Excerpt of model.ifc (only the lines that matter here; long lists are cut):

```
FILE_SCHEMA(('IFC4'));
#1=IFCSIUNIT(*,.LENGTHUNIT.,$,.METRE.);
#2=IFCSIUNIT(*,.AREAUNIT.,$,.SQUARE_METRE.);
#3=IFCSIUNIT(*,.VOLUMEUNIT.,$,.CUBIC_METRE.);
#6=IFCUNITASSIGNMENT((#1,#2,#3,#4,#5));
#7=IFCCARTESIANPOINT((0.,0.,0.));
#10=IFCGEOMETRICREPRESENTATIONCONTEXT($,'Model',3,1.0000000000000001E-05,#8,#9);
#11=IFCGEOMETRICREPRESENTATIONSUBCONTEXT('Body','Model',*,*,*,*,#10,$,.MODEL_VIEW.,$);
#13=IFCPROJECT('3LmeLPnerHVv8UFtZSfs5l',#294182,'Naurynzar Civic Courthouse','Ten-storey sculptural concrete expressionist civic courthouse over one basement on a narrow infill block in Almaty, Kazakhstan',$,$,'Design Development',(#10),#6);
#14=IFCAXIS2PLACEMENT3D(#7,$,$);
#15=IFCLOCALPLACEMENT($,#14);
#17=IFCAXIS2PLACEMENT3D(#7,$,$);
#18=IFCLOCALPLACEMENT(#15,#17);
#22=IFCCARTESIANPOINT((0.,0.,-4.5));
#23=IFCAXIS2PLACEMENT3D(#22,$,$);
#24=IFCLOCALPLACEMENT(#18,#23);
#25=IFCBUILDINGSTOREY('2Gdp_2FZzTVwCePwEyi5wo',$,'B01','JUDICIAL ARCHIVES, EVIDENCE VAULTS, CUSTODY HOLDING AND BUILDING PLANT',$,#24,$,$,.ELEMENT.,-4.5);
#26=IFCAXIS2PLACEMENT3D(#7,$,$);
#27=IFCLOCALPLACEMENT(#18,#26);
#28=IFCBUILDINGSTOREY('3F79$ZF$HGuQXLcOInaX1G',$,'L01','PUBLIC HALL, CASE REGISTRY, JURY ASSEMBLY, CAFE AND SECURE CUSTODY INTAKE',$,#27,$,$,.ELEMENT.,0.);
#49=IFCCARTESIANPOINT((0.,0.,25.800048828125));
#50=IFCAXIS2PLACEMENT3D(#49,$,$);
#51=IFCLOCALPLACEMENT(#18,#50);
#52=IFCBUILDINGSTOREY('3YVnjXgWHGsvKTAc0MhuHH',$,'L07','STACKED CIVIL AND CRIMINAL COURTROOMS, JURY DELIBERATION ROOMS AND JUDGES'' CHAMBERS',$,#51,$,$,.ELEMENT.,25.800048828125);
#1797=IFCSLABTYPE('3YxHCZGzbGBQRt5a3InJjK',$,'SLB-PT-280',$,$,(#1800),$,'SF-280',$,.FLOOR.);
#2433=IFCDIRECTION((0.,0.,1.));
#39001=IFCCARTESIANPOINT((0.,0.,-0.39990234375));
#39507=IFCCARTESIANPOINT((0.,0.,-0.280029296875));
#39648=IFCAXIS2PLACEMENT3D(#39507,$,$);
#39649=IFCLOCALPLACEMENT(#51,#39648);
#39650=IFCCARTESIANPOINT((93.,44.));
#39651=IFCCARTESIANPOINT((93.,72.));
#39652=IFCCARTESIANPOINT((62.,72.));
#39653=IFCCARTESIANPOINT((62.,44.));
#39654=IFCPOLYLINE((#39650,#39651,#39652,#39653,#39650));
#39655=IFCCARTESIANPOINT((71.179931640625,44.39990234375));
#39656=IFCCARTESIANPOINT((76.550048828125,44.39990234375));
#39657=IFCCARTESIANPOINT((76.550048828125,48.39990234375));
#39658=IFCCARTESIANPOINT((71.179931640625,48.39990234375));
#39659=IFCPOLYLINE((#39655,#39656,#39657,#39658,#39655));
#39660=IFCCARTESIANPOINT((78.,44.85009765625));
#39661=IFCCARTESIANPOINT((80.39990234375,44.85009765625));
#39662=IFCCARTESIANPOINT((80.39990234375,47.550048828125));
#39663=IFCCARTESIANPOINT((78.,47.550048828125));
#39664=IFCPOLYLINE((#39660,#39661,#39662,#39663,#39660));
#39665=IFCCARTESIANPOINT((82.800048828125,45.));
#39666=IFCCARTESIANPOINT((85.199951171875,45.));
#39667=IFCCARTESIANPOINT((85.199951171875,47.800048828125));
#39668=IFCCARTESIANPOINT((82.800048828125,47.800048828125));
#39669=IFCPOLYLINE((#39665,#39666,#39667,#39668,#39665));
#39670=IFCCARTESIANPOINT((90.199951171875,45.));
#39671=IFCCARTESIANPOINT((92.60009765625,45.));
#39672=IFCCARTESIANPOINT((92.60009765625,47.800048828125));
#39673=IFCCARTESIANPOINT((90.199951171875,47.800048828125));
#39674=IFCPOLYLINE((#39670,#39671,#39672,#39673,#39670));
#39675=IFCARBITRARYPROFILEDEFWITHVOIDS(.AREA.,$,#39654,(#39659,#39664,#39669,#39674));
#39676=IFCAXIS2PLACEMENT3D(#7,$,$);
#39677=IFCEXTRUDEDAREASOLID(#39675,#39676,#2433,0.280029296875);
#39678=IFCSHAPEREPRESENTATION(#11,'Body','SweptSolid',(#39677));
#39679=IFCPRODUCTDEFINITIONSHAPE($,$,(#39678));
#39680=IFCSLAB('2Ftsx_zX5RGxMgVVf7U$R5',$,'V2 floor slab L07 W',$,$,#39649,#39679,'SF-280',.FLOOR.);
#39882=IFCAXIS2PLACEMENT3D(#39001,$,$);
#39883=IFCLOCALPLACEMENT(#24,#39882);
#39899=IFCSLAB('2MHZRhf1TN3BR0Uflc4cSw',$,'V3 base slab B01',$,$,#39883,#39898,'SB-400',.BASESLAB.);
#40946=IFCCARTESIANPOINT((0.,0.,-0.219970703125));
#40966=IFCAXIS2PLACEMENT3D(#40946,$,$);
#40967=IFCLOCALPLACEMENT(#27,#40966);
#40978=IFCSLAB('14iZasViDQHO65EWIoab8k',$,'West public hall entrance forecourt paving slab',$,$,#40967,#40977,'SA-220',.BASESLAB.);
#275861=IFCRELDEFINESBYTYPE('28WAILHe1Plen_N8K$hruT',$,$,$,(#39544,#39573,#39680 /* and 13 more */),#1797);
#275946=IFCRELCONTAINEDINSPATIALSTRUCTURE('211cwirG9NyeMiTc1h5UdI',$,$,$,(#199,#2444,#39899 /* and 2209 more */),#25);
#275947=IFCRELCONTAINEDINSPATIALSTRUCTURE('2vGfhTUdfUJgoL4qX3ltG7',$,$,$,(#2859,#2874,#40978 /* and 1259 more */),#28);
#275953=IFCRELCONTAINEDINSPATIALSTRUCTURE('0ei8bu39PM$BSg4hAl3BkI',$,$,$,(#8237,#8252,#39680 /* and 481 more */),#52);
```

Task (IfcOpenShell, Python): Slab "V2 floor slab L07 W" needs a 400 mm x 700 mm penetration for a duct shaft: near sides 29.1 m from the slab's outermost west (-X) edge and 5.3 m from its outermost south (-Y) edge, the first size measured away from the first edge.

```python
import numpy as np
import ifcopenshell
import ifcopenshell.api.feature
import ifcopenshell.api.geometry
import ifcopenshell.api.root
import ifcopenshell.geom
import ifcopenshell.util.placement
import ifcopenshell.util.representation
import ifcopenshell.util.shape
import ifcopenshell.util.unit

model = ifcopenshell.open("model.ifc")
unit_scale = ifcopenshell.util.unit.calculate_unit_scale(model)
settings = ifcopenshell.geom.settings()


def volume(element):
    """Net volume in cubic metres, openings subtracted."""
    shape = ifcopenshell.geom.create_shape(settings, element)
    return ifcopenshell.util.shape.get_volume(shape.geometry)


slab = model.by_guid("2Ftsx_zX5RGxMgVVf7U$R5")
before = volume(slab)

# Extent in the slab's own axes, in metres. The edges named are its -X and -Y sides.
slab_shape = ifcopenshell.geom.create_shape(settings, slab)
vertices = ifcopenshell.util.shape.get_vertices(slab_shape.geometry)
x_min, y_min, bottom = vertices.min(axis=0)
top = vertices[:, 2].max()

opening = ifcopenshell.api.root.create_entity(model, ifc_class="IfcOpeningElement", name="Duct shaft opening", predefined_type="OPENING")
context = ifcopenshell.util.representation.get_context(model, "Model", "Body", "MODEL_VIEW")
width, depth = 0.4, 0.7
outline = [(0.0, 0.0), (width, 0.0), (width, depth), (0.0, depth), (0.0, 0.0)]
# Overshoot both faces by 50 mm so the cut is clean.
shape = ifcopenshell.api.geometry.add_slab_representation(
    model, context=context, depth=top - bottom + 0.1, polyline=outline
)
ifcopenshell.api.geometry.assign_representation(model, product=opening, representation=shape)

matrix = ifcopenshell.util.placement.get_local_placement(slab.ObjectPlacement)
matrix[:, 3] = matrix @ np.append(np.array([x_min + 29.1, y_min + 5.3, bottom - 0.05]) / unit_scale, 1.0)
ifcopenshell.api.geometry.edit_object_placement(model, product=opening, matrix=matrix, is_si=False)
ifcopenshell.api.feature.add_feature(model, feature=opening, element=slab)

after = volume(slab)

print(f"slab volume {before:.3f} -> {after:.3f} m3")

model.write("model_updated.ifc")
```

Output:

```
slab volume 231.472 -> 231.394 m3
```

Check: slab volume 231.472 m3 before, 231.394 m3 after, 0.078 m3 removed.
